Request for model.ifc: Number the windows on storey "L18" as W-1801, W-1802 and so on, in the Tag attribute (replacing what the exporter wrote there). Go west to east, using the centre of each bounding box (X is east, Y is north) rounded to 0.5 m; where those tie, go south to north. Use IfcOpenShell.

First a look at what the model holds.

```python
import ifcopenshell
import ifcopenshell.util.element
import ifcopenshell.util.placement

model = ifcopenshell.open("model.ifc")
print(model.schema)
storey = next(s for s in model.by_type("IfcBuildingStorey") if s.Name == "L18")
windows = [e for e in ifcopenshell.util.element.get_decomposition(storey) if e.is_a("IfcWindow")]
for e in sorted(windows, key=lambda e: e.id()):
    origin = ifcopenshell.util.placement.get_local_placement(e.ObjectPlacement)[:3, 3]
    print(e.id(), e.Tag, e.Name, origin.round(2) + 0.0, sep=" | ")
```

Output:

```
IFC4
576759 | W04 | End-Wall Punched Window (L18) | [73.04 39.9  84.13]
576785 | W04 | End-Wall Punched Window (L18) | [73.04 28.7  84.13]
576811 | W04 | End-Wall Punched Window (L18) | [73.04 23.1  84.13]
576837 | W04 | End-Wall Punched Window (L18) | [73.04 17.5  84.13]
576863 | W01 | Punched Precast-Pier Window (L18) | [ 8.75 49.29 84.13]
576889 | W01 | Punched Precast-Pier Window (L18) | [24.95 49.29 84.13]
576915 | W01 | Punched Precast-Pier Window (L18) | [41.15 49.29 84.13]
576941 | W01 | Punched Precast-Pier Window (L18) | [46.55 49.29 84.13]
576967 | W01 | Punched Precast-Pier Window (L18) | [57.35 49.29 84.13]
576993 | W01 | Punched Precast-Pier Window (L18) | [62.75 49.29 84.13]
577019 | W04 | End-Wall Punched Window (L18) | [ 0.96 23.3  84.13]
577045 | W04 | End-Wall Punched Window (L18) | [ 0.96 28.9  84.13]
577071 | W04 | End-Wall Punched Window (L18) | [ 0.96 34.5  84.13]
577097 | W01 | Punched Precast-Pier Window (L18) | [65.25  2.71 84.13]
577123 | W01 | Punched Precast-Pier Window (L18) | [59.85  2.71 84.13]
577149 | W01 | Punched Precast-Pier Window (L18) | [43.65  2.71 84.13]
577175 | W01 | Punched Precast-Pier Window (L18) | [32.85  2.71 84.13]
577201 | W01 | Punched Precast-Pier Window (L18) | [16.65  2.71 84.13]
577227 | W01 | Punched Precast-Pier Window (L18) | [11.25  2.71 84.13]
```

```python
import ifcopenshell
import ifcopenshell.geom
import ifcopenshell.util.element
import ifcopenshell.util.shape

model = ifcopenshell.open("model.ifc")
settings = ifcopenshell.geom.settings()
settings.set("use-world-coords", True)


def centre(element):
    shape = ifcopenshell.geom.create_shape(settings, element)
    return ifcopenshell.util.shape.get_bbox_centroid(shape.geometry)


storey = next(s for s in model.by_type("IfcBuildingStorey") if s.Name == "L18")
windows = [e for e in ifcopenshell.util.element.get_decomposition(storey) if e.is_a("IfcWindow")]

# Insertion points can sit at a corner or the storey origin, so sort by the geometry (in metres).
centres = {e: centre(e) for e in windows}
windows.sort(key=lambda e: (round(centres[e][0] / 0.5), centres[e][1]))

for i, e in enumerate(windows, start=1):
    number = f"W-18{i:02d}"
    e.Tag = number
    print(e.id(), number)

model.write("model_rev.ifc")
```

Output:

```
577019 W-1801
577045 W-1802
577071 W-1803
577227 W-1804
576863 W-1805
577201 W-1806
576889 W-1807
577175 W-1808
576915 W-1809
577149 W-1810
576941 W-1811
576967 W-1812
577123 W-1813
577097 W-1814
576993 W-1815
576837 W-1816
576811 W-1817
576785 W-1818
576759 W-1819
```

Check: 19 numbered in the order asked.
